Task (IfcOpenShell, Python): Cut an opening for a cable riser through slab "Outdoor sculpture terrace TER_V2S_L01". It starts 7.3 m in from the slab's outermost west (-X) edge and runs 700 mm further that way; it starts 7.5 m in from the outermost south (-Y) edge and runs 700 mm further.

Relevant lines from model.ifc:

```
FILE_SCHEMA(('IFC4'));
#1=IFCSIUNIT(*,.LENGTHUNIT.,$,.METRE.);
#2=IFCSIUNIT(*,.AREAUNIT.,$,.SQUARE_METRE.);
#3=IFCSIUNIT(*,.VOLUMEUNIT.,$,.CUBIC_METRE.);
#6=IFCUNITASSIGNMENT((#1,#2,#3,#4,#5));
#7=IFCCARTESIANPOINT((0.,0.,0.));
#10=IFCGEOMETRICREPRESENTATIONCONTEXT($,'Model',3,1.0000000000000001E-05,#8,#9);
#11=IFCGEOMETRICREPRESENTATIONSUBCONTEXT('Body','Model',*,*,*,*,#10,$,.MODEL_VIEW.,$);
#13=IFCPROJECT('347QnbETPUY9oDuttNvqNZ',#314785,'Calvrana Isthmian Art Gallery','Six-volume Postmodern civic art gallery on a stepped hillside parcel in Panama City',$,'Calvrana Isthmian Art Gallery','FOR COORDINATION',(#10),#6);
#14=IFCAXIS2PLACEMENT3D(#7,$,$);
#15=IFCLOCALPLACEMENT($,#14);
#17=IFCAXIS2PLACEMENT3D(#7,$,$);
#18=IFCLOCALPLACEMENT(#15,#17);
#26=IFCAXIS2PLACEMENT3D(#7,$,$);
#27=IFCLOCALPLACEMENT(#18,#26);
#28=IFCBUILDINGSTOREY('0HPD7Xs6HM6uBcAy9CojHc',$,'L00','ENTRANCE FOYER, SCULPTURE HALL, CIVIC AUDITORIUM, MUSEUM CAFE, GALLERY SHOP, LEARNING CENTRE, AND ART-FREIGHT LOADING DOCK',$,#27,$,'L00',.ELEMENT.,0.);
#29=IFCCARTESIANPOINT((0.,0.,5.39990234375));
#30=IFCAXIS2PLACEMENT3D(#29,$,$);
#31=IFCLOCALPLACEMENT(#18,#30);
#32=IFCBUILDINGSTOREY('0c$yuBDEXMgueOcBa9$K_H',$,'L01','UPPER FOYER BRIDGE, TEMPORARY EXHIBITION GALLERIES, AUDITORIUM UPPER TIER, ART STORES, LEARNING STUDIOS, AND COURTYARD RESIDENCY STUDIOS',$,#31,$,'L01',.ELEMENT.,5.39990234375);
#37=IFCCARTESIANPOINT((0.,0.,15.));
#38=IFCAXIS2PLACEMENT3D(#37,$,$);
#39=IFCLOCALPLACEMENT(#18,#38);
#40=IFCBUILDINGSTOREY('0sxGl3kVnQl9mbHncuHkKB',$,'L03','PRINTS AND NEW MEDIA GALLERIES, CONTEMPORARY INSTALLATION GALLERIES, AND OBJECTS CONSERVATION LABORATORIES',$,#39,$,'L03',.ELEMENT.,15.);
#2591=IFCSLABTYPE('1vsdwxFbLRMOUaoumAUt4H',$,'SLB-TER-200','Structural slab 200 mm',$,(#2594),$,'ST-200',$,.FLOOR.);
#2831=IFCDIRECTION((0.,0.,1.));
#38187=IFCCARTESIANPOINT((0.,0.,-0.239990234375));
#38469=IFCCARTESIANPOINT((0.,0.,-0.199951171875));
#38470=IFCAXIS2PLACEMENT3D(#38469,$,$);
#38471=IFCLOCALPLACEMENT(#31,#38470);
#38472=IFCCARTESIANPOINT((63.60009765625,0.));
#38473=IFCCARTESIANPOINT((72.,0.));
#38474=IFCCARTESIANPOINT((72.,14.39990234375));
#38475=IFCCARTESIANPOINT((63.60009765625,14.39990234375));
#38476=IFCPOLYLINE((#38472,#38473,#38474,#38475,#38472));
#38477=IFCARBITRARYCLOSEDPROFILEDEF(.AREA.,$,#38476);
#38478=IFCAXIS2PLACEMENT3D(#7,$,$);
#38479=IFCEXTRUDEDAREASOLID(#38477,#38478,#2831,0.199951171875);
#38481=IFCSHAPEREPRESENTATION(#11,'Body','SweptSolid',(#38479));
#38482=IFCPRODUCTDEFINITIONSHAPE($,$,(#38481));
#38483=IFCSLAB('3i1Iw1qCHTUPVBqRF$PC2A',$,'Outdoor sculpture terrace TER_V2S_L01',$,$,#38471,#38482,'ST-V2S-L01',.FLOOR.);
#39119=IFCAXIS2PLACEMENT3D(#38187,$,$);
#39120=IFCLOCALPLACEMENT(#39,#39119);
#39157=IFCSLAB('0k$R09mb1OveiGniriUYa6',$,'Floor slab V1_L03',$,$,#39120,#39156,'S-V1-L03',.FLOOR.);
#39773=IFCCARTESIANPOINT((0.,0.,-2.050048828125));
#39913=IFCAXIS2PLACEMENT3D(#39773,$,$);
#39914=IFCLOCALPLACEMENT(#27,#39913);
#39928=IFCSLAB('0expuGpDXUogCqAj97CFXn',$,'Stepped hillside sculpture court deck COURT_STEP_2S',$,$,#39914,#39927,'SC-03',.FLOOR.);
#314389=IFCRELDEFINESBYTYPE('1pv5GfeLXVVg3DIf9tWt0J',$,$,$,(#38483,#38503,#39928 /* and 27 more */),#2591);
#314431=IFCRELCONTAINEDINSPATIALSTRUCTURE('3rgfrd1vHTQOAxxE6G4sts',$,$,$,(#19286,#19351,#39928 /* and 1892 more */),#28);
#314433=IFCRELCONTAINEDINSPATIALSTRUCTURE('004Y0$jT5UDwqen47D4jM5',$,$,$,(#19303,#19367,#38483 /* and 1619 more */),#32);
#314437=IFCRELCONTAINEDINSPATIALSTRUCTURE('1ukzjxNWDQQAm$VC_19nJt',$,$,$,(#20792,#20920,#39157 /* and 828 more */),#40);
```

```python
import numpy as np
import ifcopenshell
import ifcopenshell.api.feature
import ifcopenshell.api.geometry
import ifcopenshell.api.root
import ifcopenshell.geom
import ifcopenshell.util.placement
import ifcopenshell.util.representation
import ifcopenshell.util.shape
import ifcopenshell.util.unit

model = ifcopenshell.open("model.ifc")
unit_scale = ifcopenshell.util.unit.calculate_unit_scale(model)
settings = ifcopenshell.geom.settings()


def volume(element):
    """Net volume in cubic metres, openings subtracted."""
    shape = ifcopenshell.geom.create_shape(settings, element)
    return ifcopenshell.util.shape.get_volume(shape.geometry)


slab = model.by_guid("3i1Iw1qCHTUPVBqRF$PC2A")
before = volume(slab)

# Extent in the slab's own axes, in metres. The edges named are its -X and -Y sides.
slab_shape = ifcopenshell.geom.create_shape(settings, slab)
vertices = ifcopenshell.util.shape.get_vertices(slab_shape.geometry)
x_min, y_min, bottom = vertices.min(axis=0)
top = vertices[:, 2].max()

opening = ifcopenshell.api.root.create_entity(model, ifc_class="IfcOpeningElement", name="Cable riser opening", predefined_type="OPENING")
context = ifcopenshell.util.representation.get_context(model, "Model", "Body", "MODEL_VIEW")
width, depth = 0.7, 0.7
outline = [(0.0, 0.0), (width, 0.0), (width, depth), (0.0, depth), (0.0, 0.0)]
# Overshoot both faces by 50 mm so the cut is clean.
shape = ifcopenshell.api.geometry.add_slab_representation(
    model, context=context, depth=top - bottom + 0.1, polyline=outline
)
ifcopenshell.api.geometry.assign_representation(model, product=opening, representation=shape)

matrix = ifcopenshell.util.placement.get_local_placement(slab.ObjectPlacement)
matrix[:, 3] = matrix @ np.append(np.array([x_min + 7.3, y_min + 7.5, bottom - 0.05]) / unit_scale, 1.0)
ifcopenshell.api.geometry.edit_object_placement(model, product=opening, matrix=matrix, is_si=False)
ifcopenshell.api.feature.add_feature(model, feature=opening, element=slab)

after = volume(slab)

print(f"slab volume {before:.3f} -> {after:.3f} m3")

model.write("model_v2.ifc")
```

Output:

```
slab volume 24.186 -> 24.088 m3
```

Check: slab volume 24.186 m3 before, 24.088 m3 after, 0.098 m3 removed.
